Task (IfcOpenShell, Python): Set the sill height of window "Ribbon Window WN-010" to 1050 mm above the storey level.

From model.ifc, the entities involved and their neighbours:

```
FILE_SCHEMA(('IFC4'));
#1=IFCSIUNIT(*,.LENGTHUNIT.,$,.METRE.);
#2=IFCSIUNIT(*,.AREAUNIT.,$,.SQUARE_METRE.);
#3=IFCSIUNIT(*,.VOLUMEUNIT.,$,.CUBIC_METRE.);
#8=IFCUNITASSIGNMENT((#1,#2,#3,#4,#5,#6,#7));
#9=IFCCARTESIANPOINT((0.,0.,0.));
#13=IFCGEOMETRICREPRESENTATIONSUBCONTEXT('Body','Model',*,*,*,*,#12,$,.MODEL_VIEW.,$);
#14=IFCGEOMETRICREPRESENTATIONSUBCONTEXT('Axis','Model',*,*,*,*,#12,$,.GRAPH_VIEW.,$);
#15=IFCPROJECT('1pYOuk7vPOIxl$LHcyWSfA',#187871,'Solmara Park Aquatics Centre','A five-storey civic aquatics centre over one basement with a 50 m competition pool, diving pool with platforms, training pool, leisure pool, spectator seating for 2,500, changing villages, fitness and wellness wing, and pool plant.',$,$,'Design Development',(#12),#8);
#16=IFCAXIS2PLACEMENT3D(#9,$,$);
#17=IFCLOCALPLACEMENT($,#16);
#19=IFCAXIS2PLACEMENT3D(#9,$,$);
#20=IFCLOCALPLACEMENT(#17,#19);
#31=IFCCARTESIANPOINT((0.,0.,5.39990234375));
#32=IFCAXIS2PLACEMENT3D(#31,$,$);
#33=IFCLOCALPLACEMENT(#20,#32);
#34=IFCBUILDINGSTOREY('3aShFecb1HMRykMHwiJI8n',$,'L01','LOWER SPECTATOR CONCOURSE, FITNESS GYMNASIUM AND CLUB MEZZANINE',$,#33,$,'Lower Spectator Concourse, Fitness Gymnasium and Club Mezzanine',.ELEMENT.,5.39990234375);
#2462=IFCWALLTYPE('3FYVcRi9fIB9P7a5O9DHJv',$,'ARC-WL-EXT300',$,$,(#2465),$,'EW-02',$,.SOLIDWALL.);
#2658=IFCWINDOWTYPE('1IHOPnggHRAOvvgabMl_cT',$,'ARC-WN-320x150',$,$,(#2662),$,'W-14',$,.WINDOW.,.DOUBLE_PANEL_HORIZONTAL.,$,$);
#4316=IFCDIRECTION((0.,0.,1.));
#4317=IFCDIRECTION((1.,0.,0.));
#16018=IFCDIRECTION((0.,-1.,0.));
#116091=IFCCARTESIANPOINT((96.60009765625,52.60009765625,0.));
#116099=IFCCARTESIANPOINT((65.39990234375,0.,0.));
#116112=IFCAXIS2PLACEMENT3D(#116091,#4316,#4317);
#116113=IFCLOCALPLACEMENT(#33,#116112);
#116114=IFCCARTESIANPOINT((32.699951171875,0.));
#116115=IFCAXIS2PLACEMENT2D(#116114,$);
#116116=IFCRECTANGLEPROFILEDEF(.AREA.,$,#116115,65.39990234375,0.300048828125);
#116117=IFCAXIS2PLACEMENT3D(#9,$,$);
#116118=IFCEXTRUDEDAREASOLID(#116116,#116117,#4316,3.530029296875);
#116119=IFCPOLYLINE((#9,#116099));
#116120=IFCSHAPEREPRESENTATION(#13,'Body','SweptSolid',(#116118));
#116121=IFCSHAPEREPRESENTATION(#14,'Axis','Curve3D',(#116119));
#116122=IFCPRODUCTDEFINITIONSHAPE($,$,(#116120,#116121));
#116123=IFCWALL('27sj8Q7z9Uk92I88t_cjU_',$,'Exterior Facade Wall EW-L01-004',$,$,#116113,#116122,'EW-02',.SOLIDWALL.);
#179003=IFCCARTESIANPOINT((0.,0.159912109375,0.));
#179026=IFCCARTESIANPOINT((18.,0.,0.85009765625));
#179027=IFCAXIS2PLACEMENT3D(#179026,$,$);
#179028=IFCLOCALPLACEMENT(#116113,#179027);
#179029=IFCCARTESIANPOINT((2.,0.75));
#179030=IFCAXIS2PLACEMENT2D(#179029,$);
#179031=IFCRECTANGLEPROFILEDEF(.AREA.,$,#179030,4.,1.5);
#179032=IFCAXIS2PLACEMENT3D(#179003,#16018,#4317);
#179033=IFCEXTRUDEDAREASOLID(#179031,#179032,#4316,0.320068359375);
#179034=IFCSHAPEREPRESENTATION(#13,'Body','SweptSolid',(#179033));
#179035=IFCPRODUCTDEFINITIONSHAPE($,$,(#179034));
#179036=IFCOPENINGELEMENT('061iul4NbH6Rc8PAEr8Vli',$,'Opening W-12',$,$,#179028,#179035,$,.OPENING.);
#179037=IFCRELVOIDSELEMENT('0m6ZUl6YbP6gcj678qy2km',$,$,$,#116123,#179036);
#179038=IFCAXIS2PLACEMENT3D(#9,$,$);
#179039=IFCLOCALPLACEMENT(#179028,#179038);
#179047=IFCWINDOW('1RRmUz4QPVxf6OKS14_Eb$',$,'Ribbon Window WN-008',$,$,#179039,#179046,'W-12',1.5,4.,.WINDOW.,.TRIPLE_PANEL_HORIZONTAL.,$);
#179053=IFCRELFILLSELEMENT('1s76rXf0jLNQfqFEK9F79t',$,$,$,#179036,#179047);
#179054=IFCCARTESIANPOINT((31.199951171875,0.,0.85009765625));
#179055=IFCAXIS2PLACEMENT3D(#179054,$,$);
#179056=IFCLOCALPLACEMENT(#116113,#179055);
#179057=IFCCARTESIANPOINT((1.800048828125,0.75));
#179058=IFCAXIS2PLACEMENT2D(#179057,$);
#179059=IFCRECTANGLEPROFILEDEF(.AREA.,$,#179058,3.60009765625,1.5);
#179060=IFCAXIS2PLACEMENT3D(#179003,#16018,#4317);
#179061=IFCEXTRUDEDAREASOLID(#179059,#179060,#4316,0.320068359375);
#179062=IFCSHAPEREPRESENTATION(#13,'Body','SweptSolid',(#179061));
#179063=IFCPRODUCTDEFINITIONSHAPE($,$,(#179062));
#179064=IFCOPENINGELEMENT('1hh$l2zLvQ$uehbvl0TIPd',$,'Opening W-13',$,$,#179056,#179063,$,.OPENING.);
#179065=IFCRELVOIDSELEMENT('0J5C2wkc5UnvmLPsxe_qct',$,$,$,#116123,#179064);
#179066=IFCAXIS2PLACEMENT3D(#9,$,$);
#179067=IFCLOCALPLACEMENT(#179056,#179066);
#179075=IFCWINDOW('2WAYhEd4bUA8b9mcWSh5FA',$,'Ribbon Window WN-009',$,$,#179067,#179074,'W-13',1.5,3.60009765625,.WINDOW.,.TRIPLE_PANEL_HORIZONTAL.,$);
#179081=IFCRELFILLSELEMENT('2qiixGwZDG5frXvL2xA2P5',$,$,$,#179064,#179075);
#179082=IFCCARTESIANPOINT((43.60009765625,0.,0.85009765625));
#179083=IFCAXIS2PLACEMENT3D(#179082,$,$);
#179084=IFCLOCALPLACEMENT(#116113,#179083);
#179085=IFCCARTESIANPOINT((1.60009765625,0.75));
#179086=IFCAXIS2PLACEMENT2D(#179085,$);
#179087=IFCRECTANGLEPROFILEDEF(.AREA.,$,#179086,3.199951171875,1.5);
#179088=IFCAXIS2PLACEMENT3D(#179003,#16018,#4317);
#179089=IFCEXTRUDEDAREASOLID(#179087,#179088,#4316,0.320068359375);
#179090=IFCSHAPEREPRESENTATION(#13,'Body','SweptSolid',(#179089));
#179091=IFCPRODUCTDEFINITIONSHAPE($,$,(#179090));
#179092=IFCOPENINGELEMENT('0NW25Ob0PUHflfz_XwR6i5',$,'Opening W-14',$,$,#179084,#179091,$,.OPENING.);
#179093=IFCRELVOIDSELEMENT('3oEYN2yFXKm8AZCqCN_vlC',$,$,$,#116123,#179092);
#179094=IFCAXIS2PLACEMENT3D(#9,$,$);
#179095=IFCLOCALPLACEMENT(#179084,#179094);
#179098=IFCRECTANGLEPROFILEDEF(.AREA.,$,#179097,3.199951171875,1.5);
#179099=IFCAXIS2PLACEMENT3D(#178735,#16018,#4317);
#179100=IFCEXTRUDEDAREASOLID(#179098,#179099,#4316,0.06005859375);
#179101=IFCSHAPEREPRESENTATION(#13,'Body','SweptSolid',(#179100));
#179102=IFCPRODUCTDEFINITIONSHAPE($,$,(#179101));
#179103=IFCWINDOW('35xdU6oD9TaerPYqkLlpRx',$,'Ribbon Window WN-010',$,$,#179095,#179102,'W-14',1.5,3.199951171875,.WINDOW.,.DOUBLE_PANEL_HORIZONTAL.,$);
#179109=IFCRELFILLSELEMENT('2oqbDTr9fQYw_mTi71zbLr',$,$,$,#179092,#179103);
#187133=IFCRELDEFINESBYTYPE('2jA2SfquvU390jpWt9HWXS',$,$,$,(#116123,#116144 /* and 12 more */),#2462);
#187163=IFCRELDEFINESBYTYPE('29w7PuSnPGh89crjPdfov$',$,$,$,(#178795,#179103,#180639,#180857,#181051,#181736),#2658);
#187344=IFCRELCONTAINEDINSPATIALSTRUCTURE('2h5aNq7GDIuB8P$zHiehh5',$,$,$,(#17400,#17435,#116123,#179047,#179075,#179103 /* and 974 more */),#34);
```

```python
import numpy as np
import ifcopenshell
import ifcopenshell.api.geometry
import ifcopenshell.geom
import ifcopenshell.util.element
import ifcopenshell.util.placement
import ifcopenshell.util.shape
import ifcopenshell.util.unit

model = ifcopenshell.open("model.ifc")
unit_scale = ifcopenshell.util.unit.calculate_unit_scale(model)

window = model.by_id(179103)
opening = window.FillsVoids[0].RelatingOpeningElement
storey = ifcopenshell.util.element.get_container(window, ifc_class="IfcBuildingStorey")
level = ifcopenshell.util.placement.get_local_placement(storey.ObjectPlacement)[2, 3]

# The opening's origin need not be at the sill, so measure its lowest point.
shape = ifcopenshell.geom.create_shape(ifcopenshell.geom.settings(), opening)
bottom = ifcopenshell.util.shape.get_shape_bottom_elevation(shape, shape.geometry) / unit_scale
dz = level + 1.05 / unit_scale - bottom

shift = np.array([0.0, 0.0, dz])
# The window is placed relative to its opening, so it follows when the opening moves.
matrix = ifcopenshell.util.placement.get_local_placement(opening.ObjectPlacement)
matrix[:3, 3] += shift
ifcopenshell.api.geometry.edit_object_placement(
    model, product=opening, matrix=matrix, is_si=False, should_transform_children=True
)

print(f"moved by {dz * unit_scale:+.3f} m")

model.write("model_updated.ifc")
```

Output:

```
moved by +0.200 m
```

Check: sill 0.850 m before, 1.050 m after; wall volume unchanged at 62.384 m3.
